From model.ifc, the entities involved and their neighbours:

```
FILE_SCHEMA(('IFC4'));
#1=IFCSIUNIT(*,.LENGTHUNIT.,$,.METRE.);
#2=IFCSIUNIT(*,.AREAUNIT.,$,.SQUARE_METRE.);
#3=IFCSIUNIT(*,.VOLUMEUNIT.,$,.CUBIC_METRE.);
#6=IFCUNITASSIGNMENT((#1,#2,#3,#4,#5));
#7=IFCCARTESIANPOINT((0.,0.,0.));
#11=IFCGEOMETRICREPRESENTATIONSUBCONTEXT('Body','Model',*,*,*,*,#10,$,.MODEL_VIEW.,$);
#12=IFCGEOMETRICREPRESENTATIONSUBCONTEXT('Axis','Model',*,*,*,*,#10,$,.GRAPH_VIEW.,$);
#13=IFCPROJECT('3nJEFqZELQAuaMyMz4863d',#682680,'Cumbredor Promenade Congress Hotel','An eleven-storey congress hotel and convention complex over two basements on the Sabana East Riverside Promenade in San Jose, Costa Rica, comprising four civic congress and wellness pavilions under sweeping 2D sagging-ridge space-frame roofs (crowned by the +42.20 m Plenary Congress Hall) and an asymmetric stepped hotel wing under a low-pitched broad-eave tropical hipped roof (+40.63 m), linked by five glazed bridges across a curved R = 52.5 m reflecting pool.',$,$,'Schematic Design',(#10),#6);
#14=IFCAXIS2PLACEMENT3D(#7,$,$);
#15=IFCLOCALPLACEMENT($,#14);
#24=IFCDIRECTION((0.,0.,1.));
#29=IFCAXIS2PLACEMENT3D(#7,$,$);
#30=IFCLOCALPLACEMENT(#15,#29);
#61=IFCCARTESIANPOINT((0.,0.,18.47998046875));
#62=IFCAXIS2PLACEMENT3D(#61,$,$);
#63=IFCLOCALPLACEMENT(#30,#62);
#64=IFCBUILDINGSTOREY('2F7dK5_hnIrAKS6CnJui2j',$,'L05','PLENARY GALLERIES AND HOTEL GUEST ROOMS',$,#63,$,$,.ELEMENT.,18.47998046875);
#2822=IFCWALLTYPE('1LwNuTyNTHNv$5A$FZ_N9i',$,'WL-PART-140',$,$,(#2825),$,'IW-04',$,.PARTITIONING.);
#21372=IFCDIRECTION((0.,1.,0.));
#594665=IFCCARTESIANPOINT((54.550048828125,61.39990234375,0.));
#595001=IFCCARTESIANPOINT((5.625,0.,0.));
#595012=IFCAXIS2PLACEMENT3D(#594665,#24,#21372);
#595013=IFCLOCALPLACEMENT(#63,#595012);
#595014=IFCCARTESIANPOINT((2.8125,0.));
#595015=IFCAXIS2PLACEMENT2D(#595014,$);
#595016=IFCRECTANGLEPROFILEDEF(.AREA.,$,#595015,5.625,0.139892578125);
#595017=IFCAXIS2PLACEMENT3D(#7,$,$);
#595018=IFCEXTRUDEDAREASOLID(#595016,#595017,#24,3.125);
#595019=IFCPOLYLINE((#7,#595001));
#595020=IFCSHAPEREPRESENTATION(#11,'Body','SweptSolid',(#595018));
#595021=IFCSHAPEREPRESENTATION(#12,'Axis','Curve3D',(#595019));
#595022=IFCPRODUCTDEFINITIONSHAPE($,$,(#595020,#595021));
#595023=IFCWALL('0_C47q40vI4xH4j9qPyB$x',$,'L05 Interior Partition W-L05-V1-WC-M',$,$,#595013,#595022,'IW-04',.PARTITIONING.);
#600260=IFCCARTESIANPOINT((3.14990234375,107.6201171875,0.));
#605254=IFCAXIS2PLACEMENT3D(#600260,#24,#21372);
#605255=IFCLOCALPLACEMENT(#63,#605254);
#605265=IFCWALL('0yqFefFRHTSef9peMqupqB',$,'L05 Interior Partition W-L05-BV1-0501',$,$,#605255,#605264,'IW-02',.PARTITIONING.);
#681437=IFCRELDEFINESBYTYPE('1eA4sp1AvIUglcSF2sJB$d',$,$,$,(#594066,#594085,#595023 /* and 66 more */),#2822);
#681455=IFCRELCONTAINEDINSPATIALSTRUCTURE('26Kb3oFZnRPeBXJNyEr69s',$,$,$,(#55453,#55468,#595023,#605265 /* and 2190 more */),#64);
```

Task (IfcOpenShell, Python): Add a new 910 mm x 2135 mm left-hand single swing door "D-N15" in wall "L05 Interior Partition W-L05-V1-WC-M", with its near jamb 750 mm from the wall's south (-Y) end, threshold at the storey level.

```python
import numpy as np
import ifcopenshell
import ifcopenshell.api.feature
import ifcopenshell.api.geometry
import ifcopenshell.api.root
import ifcopenshell.api.spatial
import ifcopenshell.geom
import ifcopenshell.util.element
import ifcopenshell.util.placement
import ifcopenshell.util.representation
import ifcopenshell.util.shape
import ifcopenshell.util.unit

model = ifcopenshell.open("model.ifc")
unit_scale = ifcopenshell.util.unit.calculate_unit_scale(model)
settings = ifcopenshell.geom.settings()


def volume(element):
    """Net volume in cubic metres, openings subtracted."""
    shape = ifcopenshell.geom.create_shape(settings, element)
    return ifcopenshell.util.shape.get_volume(shape.geometry)


wall = model.by_guid("0_C47q40vI4xH4j9qPyB$x")
storey = ifcopenshell.util.element.get_container(wall, ifc_class="IfcBuildingStorey")
context = ifcopenshell.util.representation.get_context(model, "Model", "Body", "MODEL_VIEW")
before = volume(wall)

width, height, from_end, sill = 0.91, 2.135, 0.75, 0.0  # metres

# The wall runs along its own X axis, and the end named is its -X end.
wall_shape = ifcopenshell.geom.create_shape(settings, wall)
x, y, z = ifcopenshell.util.shape.get_vertices(wall_shape.geometry).T
start = x.min() + from_end
face, thickness = float(y.min()), float(y.max() - y.min())
wall_matrix = ifcopenshell.util.placement.get_local_placement(wall.ObjectPlacement)
level = ifcopenshell.util.placement.get_local_placement(storey.ObjectPlacement)[2, 3]


def in_wall(x, y):
    """Placement at x, y metres in the wall's axes, at sill height."""
    matrix = wall_matrix.copy()
    matrix[:, 3] = wall_matrix @ np.array([x / unit_scale, y / unit_scale, 0.0, 1.0])
    matrix[2, 3] = level + sill / unit_scale
    return matrix


# Opening: a box that overshoots both wall faces by 50 mm.
opening = ifcopenshell.api.root.create_entity(model, ifc_class="IfcOpeningElement", predefined_type="OPENING")
box = ifcopenshell.api.geometry.add_wall_representation(
    model, context=context, length=width, height=height, thickness=thickness + 0.1
)
ifcopenshell.api.geometry.assign_representation(model, product=opening, representation=box)
ifcopenshell.api.geometry.edit_object_placement(model, product=opening, matrix=in_wall(start, face - 0.05), is_si=False)
ifcopenshell.api.feature.add_feature(model, feature=opening, element=wall)

door = ifcopenshell.api.root.create_entity(model, ifc_class="IfcDoor", name="D-N15", predefined_type="DOOR")
door.OverallWidth, door.OverallHeight = width / unit_scale, height / unit_scale
door.OperationType = "SINGLE_SWING_LEFT"
body = ifcopenshell.api.geometry.add_door_representation(
    model,
    context=context,
    overall_width=door.OverallWidth,
    overall_height=door.OverallHeight,
    operation_type="SINGLE_SWING_LEFT",
    lining_properties={"LiningDepth": thickness / unit_scale, "ThresholdDepth": thickness / unit_scale},
)
ifcopenshell.api.geometry.assign_representation(model, product=door, representation=body)
ifcopenshell.api.spatial.assign_container(model, products=[door], relating_structure=storey)
ifcopenshell.api.feature.add_filling(model, opening=opening, element=door)

# The lining spans the wall, so the door starts at the wall face.
ifcopenshell.api.geometry.edit_object_placement(model, product=door, matrix=in_wall(start, face), is_si=False)

after = volume(wall)

print(f"wall volume {before:.3f} -> {after:.3f} m3")

model.write("model-out.ifc")
```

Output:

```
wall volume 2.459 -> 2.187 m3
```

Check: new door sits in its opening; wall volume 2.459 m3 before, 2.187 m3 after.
